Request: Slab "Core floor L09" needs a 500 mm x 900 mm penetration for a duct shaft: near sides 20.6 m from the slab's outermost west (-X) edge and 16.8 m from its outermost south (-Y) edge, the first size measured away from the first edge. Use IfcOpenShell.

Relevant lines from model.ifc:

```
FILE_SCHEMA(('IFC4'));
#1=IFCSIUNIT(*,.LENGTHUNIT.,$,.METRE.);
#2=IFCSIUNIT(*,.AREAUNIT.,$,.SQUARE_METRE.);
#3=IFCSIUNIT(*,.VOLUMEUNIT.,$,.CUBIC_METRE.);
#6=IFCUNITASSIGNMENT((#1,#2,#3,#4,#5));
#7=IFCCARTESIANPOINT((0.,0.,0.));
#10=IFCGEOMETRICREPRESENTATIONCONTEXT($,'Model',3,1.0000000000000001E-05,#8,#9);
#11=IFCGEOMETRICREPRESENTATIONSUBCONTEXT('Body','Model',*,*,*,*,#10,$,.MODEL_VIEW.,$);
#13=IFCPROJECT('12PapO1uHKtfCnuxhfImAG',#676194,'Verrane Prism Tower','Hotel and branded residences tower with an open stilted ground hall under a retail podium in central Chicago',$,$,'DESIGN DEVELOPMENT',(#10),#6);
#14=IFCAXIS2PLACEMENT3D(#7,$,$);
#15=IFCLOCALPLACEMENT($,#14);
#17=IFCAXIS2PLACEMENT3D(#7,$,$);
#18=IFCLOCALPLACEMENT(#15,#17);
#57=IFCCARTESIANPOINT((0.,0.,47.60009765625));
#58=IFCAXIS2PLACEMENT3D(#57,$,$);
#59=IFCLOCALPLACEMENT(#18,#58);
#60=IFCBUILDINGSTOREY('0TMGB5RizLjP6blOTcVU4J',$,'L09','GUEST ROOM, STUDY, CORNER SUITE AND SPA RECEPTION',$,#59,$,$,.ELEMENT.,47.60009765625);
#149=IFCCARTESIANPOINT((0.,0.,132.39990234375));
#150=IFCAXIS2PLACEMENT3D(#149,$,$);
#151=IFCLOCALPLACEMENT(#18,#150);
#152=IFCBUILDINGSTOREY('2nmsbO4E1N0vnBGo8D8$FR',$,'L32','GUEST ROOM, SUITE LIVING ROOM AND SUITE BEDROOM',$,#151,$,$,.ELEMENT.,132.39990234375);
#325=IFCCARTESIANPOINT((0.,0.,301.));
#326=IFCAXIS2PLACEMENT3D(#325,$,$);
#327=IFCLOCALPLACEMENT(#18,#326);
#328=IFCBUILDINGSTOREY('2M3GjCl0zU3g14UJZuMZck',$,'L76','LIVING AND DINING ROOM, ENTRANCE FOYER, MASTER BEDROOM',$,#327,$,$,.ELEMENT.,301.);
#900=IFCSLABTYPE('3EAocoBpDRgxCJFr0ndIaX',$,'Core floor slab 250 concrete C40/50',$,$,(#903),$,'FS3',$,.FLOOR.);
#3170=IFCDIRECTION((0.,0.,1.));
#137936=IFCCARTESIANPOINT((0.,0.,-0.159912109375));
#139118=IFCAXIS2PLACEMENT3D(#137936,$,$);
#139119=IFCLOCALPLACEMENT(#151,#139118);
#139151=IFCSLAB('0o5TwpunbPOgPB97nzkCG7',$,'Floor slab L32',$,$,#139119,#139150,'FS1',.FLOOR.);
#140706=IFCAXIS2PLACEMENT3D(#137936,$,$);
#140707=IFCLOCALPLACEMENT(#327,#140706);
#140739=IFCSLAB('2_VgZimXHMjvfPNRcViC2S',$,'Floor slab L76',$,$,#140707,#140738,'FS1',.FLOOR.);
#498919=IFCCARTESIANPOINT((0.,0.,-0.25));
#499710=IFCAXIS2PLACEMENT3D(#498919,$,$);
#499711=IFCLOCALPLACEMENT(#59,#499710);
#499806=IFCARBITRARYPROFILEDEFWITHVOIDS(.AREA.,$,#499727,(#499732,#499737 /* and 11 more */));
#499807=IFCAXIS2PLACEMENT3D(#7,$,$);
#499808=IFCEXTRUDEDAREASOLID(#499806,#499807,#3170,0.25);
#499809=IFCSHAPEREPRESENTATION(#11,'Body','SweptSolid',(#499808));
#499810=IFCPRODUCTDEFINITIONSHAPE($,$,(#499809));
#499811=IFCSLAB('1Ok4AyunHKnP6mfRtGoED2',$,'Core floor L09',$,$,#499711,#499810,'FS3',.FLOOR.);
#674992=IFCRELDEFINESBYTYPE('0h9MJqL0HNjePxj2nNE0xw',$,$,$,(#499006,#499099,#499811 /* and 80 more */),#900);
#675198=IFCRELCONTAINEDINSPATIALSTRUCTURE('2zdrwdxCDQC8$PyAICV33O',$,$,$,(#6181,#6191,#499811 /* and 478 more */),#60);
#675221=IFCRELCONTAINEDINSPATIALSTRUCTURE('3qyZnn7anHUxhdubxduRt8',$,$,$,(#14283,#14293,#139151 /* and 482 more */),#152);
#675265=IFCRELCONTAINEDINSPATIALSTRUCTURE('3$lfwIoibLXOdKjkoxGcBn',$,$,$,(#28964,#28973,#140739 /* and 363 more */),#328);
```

```python
import numpy as np
import ifcopenshell
import ifcopenshell.api.feature
import ifcopenshell.api.geometry
import ifcopenshell.api.root
import ifcopenshell.geom
import ifcopenshell.util.placement
import ifcopenshell.util.representation
import ifcopenshell.util.shape
import ifcopenshell.util.unit

model = ifcopenshell.open("model.ifc")
unit_scale = ifcopenshell.util.unit.calculate_unit_scale(model)
settings = ifcopenshell.geom.settings()


def volume(element):
    """Net volume in cubic metres, openings subtracted."""
    shape = ifcopenshell.geom.create_shape(settings, element)
    return ifcopenshell.util.shape.get_volume(shape.geometry)


slab = model.by_id(499811)
before = volume(slab)

# Extent in the slab's own axes, in metres. The edges named are its -X and -Y sides.
slab_shape = ifcopenshell.geom.create_shape(settings, slab)
vertices = ifcopenshell.util.shape.get_vertices(slab_shape.geometry)
x_min, y_min, bottom = vertices.min(axis=0)
top = vertices[:, 2].max()

opening = ifcopenshell.api.root.create_entity(model, ifc_class="IfcOpeningElement", name="Duct shaft opening", predefined_type="OPENING")
context = ifcopenshell.util.representation.get_context(model, "Model", "Body", "MODEL_VIEW")
width, depth = 0.5, 0.9
outline = [(0.0, 0.0), (width, 0.0), (width, depth), (0.0, depth), (0.0, 0.0)]
# Overshoot both faces by 50 mm so the cut is clean.
shape = ifcopenshell.api.geometry.add_slab_representation(
    model, context=context, depth=top - bottom + 0.1, polyline=outline
)
ifcopenshell.api.geometry.assign_representation(model, product=opening, representation=shape)

matrix = ifcopenshell.util.placement.get_local_placement(slab.ObjectPlacement)
matrix[:, 3] = matrix @ np.append(np.array([x_min + 20.6, y_min + 16.8, bottom - 0.05]) / unit_scale, 1.0)
ifcopenshell.api.geometry.edit_object_placement(model, product=opening, matrix=matrix, is_si=False)
ifcopenshell.api.feature.add_feature(model, feature=opening, element=slab)

after = volume(slab)

print(f"slab volume {before:.3f} -> {after:.3f} m3")

model.write("model_updated.ifc")
```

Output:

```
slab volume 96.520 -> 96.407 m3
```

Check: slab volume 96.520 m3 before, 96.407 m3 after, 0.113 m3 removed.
